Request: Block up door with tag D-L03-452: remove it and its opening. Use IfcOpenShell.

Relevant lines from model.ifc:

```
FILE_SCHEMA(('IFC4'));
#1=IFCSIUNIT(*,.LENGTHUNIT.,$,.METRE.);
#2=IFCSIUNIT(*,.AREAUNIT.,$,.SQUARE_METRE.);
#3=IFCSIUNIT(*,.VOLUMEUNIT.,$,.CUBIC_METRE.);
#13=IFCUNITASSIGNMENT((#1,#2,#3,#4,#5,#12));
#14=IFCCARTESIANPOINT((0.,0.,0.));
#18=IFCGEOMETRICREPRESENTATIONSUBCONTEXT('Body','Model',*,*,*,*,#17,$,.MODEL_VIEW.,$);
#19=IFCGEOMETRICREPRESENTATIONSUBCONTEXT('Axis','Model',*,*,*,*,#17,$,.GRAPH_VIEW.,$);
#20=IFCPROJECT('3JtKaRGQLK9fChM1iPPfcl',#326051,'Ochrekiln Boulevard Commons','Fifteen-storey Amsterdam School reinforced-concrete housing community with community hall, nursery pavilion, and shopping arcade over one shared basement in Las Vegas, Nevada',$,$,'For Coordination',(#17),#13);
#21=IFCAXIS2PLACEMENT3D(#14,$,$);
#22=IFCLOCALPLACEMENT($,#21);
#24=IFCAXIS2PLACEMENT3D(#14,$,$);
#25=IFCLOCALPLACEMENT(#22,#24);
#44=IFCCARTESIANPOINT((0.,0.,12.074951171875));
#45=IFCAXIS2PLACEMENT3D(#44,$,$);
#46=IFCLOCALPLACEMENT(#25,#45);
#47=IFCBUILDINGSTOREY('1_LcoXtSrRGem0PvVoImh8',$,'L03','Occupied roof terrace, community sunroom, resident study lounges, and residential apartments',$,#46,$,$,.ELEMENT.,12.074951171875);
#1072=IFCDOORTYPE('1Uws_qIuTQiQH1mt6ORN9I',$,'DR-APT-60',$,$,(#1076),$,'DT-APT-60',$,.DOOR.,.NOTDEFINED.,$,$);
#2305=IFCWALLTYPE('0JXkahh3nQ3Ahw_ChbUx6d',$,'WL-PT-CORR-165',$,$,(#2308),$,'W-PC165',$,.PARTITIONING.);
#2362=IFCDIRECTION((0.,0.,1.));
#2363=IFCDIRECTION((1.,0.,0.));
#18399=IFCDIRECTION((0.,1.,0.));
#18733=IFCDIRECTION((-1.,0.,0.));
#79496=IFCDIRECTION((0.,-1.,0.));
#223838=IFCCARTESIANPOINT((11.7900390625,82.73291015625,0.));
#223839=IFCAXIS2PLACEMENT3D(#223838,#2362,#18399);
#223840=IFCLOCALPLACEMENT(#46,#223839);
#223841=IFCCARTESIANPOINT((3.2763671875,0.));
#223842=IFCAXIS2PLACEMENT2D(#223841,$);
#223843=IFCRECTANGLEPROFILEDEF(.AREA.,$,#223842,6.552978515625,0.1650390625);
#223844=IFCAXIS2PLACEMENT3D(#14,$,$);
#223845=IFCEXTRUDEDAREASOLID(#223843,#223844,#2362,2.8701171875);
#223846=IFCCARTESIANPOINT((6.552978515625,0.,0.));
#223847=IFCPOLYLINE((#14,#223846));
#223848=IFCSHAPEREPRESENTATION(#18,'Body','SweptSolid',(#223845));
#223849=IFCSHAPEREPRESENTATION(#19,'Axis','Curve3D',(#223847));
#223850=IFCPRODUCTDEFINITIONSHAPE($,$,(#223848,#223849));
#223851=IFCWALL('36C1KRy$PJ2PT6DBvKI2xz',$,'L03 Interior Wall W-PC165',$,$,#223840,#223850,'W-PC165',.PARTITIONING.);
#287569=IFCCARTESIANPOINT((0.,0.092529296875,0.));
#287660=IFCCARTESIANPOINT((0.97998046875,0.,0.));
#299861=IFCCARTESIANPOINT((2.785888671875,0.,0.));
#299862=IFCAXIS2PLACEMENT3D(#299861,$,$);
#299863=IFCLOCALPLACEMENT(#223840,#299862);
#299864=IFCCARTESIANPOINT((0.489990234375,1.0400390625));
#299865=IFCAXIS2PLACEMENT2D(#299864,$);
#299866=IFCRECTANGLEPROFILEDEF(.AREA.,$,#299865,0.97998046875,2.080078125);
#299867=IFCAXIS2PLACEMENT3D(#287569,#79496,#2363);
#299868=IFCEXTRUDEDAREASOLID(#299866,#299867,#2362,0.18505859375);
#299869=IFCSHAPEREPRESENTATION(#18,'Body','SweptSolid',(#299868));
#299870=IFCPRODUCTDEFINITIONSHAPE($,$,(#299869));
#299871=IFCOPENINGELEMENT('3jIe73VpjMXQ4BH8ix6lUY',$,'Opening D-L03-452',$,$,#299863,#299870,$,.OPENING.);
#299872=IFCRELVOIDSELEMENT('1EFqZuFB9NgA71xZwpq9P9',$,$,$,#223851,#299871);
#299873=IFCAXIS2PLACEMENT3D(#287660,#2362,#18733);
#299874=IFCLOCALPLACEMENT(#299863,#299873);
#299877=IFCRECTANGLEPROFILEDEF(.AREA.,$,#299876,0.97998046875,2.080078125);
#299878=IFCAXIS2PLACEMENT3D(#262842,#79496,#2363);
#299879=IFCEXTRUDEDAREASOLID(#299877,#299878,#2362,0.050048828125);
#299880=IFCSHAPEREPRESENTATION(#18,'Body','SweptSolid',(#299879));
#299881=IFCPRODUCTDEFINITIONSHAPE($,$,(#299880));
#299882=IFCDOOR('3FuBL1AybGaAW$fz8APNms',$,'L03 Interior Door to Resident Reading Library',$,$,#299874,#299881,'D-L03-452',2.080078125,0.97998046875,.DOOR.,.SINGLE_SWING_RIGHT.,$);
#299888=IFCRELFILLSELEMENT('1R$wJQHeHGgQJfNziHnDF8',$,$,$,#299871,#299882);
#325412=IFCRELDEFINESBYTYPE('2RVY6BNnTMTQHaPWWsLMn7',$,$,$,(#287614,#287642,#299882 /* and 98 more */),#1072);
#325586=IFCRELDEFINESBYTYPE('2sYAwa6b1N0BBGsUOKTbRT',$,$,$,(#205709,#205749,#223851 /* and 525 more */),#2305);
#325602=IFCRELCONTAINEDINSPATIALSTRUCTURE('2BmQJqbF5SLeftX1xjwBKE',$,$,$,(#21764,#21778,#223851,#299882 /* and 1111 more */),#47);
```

```python
import ifcopenshell
import ifcopenshell.api.feature
import ifcopenshell.api.root
import ifcopenshell.geom
import ifcopenshell.util.shape

model = ifcopenshell.open("model.ifc")
settings = ifcopenshell.geom.settings()


def volume(element):
    """Net volume in cubic metres, openings subtracted."""
    shape = ifcopenshell.geom.create_shape(settings, element)
    return ifcopenshell.util.shape.get_volume(shape.geometry)


door = model.by_guid("3FuBL1AybGaAW$fz8APNms")
opening = door.FillsVoids[0].RelatingOpeningElement
wall = opening.VoidsElements[0].RelatingBuildingElement
before = volume(wall)

ifcopenshell.api.root.remove_product(model, product=door)
ifcopenshell.api.feature.remove_feature(model, feature=opening)

after = volume(wall)

print(f"wall volume {before:.3f} -> {after:.3f} m3")

model.write("model_rev.ifc")
```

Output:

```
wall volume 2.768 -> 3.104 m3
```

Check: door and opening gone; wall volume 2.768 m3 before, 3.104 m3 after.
